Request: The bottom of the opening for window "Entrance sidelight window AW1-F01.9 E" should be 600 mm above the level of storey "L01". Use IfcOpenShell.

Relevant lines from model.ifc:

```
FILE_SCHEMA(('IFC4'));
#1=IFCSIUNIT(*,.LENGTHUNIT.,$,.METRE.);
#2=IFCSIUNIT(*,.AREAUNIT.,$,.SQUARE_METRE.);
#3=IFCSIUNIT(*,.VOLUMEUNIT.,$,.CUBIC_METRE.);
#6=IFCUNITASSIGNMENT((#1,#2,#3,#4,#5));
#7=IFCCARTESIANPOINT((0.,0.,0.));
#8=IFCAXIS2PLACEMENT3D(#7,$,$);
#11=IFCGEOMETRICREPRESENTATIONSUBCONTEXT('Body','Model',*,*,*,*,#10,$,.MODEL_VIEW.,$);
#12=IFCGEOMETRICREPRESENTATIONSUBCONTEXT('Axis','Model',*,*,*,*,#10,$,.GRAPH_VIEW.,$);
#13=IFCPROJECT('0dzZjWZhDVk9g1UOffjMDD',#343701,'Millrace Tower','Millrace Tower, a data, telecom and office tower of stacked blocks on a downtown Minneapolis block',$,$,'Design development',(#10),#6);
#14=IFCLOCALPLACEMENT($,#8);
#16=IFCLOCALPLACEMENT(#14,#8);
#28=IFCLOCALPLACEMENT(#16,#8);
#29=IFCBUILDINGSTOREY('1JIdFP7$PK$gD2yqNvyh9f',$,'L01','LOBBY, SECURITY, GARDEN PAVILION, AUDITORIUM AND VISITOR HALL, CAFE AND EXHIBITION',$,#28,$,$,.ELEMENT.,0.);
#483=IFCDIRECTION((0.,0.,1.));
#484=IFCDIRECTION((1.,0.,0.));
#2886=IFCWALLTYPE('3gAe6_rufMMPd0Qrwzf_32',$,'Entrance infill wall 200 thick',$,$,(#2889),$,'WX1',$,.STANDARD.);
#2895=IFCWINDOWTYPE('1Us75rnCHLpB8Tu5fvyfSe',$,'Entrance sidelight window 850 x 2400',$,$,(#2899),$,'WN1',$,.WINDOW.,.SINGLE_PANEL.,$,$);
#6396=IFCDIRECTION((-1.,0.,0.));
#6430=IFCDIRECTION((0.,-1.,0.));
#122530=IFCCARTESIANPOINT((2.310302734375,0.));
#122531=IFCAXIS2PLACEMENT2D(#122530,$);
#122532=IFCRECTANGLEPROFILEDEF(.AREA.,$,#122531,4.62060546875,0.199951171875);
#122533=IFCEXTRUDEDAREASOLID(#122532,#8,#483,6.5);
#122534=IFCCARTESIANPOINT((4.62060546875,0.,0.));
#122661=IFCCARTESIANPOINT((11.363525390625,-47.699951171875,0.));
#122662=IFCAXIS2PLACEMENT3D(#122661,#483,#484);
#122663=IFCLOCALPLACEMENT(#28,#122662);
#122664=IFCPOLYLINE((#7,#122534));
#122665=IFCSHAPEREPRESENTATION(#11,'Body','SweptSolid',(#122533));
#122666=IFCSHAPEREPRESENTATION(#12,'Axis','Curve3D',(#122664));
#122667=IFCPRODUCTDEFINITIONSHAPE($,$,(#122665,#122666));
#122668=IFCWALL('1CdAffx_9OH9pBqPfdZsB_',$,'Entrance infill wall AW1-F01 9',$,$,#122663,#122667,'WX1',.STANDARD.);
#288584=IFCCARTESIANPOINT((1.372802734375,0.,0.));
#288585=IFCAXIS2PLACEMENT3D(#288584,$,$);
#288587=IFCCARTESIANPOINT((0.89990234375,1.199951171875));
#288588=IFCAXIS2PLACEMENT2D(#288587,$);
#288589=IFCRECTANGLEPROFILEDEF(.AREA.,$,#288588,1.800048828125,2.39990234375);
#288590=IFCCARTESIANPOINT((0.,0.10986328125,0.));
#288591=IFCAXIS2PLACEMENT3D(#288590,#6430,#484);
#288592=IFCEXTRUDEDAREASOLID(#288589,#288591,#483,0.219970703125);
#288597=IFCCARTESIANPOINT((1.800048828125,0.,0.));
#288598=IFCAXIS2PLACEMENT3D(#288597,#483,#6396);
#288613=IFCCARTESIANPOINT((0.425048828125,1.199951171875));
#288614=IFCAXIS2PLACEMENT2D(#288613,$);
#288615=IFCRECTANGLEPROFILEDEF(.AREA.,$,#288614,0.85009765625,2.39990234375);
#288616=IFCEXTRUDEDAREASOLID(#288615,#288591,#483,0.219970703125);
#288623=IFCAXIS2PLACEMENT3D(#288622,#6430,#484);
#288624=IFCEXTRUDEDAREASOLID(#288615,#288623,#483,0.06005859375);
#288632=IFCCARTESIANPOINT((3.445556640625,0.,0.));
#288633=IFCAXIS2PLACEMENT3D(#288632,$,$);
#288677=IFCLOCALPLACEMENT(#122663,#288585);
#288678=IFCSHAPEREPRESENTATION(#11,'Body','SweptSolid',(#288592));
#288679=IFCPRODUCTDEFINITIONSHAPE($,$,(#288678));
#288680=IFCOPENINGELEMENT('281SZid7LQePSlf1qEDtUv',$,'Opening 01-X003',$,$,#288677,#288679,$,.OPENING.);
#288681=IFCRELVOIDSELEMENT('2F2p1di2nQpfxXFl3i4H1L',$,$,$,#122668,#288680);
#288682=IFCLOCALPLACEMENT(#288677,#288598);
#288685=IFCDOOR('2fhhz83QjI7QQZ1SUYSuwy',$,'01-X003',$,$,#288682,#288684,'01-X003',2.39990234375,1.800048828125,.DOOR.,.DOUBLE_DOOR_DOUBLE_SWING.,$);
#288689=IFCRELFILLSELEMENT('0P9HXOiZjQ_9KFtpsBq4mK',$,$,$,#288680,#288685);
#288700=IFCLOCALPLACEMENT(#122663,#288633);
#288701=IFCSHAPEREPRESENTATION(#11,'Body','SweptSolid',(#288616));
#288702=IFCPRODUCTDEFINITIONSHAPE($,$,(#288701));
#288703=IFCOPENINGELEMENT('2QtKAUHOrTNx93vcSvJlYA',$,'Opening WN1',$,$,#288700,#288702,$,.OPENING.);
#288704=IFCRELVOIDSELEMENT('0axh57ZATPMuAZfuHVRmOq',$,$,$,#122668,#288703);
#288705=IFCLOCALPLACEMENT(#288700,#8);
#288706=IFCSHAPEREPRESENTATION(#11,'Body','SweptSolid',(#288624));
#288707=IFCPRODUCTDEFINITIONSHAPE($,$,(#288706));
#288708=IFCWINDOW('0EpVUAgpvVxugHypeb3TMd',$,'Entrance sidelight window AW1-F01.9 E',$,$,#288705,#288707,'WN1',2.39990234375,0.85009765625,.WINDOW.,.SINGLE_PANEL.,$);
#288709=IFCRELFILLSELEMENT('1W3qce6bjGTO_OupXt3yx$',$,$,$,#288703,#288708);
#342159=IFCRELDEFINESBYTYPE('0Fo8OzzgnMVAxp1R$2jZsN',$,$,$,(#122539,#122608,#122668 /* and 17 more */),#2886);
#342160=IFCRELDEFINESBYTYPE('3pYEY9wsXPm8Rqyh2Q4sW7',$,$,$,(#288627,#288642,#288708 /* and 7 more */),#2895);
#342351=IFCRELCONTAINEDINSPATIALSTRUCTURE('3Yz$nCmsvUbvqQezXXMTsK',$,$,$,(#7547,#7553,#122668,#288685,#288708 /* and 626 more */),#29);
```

```python
import numpy as np
import ifcopenshell
import ifcopenshell.api.geometry
import ifcopenshell.geom
import ifcopenshell.util.element
import ifcopenshell.util.placement
import ifcopenshell.util.shape
import ifcopenshell.util.unit

model = ifcopenshell.open("model.ifc")
unit_scale = ifcopenshell.util.unit.calculate_unit_scale(model)

window = model.by_guid("0EpVUAgpvVxugHypeb3TMd")
opening = window.FillsVoids[0].RelatingOpeningElement
storey = ifcopenshell.util.element.get_container(window, ifc_class="IfcBuildingStorey")
level = ifcopenshell.util.placement.get_local_placement(storey.ObjectPlacement)[2, 3]

# The opening's origin need not be at the sill, so measure its lowest point.
shape = ifcopenshell.geom.create_shape(ifcopenshell.geom.settings(), opening)
bottom = ifcopenshell.util.shape.get_shape_bottom_elevation(shape, shape.geometry) / unit_scale
dz = level + 0.6 - bottom

shift = np.array([0.0, 0.0, dz])
# The window is placed relative to its opening, so it follows when the opening moves.
matrix = ifcopenshell.util.placement.get_local_placement(opening.ObjectPlacement)
matrix[:3, 3] += shift
ifcopenshell.api.geometry.edit_object_placement(
    model, product=opening, matrix=matrix, is_si=False, should_transform_children=True
)

print(f"moved by {dz * unit_scale:+.3f} m")

model.write("model_updated.ifc")
```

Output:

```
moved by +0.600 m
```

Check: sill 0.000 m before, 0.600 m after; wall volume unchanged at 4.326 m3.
